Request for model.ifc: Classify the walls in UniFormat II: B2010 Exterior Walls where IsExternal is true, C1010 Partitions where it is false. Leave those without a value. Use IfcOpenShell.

First a look at what the model holds.

```python
import ifcopenshell
import ifcopenshell.util.element

model = ifcopenshell.open("model.ifc")
print(model.schema)
print("classifications:", [c.Name for c in model.by_type("IfcClassification")])
values = [ifcopenshell.util.element.get_pset(e, "Pset_WallCommon", "IsExternal") for e in model.by_type("IfcWall")]
for value in (True, False, None):
    print("IsExternal", value, values.count(value))
```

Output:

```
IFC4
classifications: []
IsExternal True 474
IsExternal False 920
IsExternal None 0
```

```python
import ifcopenshell
import ifcopenshell.api.classification
import ifcopenshell.util.element

model = ifcopenshell.open("model.ifc")

system = ifcopenshell.api.classification.add_classification(model, classification="UniFormat II")

walls = model.by_type("IfcWall")
external = {e: ifcopenshell.util.element.get_pset(e, "Pset_WallCommon", "IsExternal") for e in walls}
for flag, code, name in ((True, "B2010", "Exterior Walls"), (False, "C1010", "Partitions")):
    products = [e for e in walls if external[e] is flag]
    ifcopenshell.api.classification.add_reference(
        model, products=products, classification=system, identification=code, name=name
    )
    print(code, len(products))

model.write("model_updated.ifc")
```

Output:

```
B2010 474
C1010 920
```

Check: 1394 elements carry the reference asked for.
